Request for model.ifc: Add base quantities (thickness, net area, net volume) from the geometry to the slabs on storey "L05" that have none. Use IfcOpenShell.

First a look at what the model holds.

```python
import ifcopenshell
import ifcopenshell.util.element
import ifcopenshell.util.unit

model = ifcopenshell.open("model.ifc")
print(model.schema)
for unit_type in ("LENGTHUNIT", "AREAUNIT", "VOLUMEUNIT"):
    print(unit_type, ifcopenshell.util.unit.calculate_unit_scale(model, unit_type))
storey = next(s for s in model.by_type("IfcBuildingStorey") if s.Name == "L05")
slabs = [e for e in ifcopenshell.util.element.get_decomposition(storey) if e.is_a("IfcSlab")]
for e in sorted(slabs, key=lambda e: e.id()):
    print(e.id(), e.is_a(), e.Name, list(ifcopenshell.util.element.get_psets(e, qtos_only=True)), sep=" | ")
```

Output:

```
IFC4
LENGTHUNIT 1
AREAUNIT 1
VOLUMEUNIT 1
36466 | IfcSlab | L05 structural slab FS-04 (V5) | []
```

```python
import ifcopenshell
import ifcopenshell.api.pset
import ifcopenshell.geom
import ifcopenshell.util.element
import ifcopenshell.util.shape
import ifcopenshell.util.unit

model = ifcopenshell.open("model.ifc")
unit_scale = ifcopenshell.util.unit.calculate_unit_scale(model)
area_scale = ifcopenshell.util.unit.calculate_unit_scale(model, "AREAUNIT")
volume_scale = ifcopenshell.util.unit.calculate_unit_scale(model, "VOLUMEUNIT")
settings = ifcopenshell.geom.settings()

storey = next(s for s in model.by_type("IfcBuildingStorey") if s.Name == "L05")
slabs = [e for e in ifcopenshell.util.element.get_decomposition(storey) if e.is_a("IfcSlab")]

for e in sorted(slabs, key=lambda e: e.id()):
    if ifcopenshell.util.element.get_psets(e, qtos_only=True, should_inherit=False):
        continue
    # Geometry comes back in metres, in the element's own axes.
    shape = ifcopenshell.geom.create_shape(settings, e)
    values = {
        "Width": ifcopenshell.util.shape.get_z(shape.geometry) / unit_scale,
        "NetArea": ifcopenshell.util.shape.get_footprint_area(shape.geometry) / area_scale,
        "NetVolume": ifcopenshell.util.shape.get_volume(shape.geometry) / volume_scale,
    }
    qto = ifcopenshell.api.pset.add_qto(model, product=e, name="Qto_SlabBaseQuantities")
    ifcopenshell.api.pset.edit_qto(model, qto=qto, properties=values)
    print(e.id(), {k: round(v, 3) for k, v in values.items()})

model.write("model_v2.ifc")
```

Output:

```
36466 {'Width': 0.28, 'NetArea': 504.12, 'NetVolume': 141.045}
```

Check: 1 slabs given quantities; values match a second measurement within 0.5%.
